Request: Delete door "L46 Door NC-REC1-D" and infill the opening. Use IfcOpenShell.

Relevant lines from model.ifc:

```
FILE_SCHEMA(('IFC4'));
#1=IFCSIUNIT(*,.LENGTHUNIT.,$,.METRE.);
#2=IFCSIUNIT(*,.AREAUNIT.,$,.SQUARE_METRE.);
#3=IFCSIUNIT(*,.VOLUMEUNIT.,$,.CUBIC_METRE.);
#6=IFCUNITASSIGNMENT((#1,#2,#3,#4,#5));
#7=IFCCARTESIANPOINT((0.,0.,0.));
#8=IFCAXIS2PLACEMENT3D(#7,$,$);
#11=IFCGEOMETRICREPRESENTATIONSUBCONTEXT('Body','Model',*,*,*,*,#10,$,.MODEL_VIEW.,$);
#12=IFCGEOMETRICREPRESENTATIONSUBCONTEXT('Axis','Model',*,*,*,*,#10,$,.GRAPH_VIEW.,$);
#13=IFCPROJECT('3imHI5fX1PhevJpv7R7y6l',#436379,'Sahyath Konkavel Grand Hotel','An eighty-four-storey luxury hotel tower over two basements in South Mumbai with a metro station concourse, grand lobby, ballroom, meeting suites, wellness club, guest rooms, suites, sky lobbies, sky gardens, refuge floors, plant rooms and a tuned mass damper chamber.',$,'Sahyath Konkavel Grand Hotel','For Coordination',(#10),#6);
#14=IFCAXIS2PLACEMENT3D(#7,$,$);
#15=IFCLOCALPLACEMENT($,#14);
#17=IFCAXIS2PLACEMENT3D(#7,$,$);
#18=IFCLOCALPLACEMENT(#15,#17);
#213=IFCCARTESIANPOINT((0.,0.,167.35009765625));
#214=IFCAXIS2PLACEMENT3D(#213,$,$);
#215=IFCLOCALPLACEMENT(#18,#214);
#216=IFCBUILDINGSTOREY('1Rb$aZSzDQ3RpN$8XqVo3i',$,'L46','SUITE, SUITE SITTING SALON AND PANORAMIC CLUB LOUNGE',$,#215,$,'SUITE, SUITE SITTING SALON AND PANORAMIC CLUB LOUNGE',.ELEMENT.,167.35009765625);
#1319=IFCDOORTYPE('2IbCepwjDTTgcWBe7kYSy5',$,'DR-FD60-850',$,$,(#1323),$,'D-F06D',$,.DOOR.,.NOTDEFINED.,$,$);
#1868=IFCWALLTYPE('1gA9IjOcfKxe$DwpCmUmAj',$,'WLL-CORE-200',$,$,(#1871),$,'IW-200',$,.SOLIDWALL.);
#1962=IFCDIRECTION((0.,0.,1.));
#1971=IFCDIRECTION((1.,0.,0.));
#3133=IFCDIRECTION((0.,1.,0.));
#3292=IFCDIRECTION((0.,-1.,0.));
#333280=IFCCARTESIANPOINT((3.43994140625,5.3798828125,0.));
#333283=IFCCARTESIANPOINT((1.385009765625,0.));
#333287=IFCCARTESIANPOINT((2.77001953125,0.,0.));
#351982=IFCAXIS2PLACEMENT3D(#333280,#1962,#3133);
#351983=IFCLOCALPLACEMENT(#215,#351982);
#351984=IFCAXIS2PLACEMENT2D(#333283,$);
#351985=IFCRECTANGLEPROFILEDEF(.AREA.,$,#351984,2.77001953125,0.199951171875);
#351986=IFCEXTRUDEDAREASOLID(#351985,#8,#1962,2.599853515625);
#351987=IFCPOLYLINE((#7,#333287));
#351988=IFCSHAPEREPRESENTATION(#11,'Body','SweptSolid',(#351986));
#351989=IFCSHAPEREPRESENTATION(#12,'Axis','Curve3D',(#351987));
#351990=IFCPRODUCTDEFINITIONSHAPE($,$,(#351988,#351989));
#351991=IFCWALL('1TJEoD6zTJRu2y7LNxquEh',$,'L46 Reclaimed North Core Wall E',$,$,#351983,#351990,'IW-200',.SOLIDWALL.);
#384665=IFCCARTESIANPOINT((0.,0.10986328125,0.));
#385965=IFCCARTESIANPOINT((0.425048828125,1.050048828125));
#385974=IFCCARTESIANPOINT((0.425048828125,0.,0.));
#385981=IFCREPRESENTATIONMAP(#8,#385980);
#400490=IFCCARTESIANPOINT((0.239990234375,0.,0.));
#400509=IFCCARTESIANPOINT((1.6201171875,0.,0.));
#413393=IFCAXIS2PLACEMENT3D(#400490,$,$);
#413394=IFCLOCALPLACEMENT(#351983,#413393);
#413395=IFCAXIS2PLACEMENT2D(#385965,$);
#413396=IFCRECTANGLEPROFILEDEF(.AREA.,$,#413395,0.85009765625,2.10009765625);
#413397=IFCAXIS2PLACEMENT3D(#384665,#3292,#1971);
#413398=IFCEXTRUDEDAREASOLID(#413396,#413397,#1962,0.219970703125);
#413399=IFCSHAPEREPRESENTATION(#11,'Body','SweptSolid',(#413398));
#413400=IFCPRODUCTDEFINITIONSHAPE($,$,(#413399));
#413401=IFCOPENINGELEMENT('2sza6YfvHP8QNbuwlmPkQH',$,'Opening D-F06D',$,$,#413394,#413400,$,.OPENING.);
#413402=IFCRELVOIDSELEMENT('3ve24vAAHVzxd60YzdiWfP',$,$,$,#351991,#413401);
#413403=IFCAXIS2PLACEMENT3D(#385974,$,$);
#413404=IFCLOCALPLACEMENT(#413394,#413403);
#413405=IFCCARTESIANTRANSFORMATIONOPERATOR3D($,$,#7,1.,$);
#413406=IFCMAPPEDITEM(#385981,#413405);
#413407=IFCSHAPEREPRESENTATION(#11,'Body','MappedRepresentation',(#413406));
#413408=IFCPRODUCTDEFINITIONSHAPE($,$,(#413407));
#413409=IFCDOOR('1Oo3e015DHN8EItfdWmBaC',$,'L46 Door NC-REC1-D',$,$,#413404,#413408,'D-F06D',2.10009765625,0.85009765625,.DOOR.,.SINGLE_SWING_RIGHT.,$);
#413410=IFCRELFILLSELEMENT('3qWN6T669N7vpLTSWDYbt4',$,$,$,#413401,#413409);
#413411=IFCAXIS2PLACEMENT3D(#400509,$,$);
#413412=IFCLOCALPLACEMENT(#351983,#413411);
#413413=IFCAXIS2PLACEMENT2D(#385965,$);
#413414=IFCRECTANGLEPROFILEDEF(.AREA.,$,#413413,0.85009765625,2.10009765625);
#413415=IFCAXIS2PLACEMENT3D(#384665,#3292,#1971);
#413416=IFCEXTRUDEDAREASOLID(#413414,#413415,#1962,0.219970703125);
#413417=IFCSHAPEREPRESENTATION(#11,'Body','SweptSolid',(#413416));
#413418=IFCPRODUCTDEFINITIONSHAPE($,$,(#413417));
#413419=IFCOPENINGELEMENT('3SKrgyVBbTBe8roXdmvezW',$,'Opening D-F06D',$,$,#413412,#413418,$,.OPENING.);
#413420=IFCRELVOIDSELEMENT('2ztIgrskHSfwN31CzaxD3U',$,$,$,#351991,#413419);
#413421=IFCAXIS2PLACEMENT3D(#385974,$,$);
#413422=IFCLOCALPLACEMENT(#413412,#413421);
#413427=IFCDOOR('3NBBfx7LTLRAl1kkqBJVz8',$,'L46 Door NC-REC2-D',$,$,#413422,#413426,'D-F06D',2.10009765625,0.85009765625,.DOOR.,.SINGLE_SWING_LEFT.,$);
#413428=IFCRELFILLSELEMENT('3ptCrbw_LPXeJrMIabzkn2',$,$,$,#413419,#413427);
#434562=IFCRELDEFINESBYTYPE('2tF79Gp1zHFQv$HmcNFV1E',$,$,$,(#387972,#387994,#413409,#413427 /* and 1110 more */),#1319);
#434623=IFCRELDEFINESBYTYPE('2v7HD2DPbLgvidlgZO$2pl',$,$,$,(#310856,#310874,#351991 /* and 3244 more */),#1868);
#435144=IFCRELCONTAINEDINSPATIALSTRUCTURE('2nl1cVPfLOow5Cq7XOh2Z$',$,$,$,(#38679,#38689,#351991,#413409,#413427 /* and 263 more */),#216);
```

```python
import ifcopenshell
import ifcopenshell.api.feature
import ifcopenshell.api.root
import ifcopenshell.geom
import ifcopenshell.util.shape

model = ifcopenshell.open("model.ifc")
settings = ifcopenshell.geom.settings()


def volume(element):
    """Net volume in cubic metres, openings subtracted."""
    shape = ifcopenshell.geom.create_shape(settings, element)
    return ifcopenshell.util.shape.get_volume(shape.geometry)


door = model.by_id(413409)
opening = door.FillsVoids[0].RelatingOpeningElement
wall = opening.VoidsElements[0].RelatingBuildingElement
before = volume(wall)

ifcopenshell.api.root.remove_product(model, product=door)
ifcopenshell.api.feature.remove_feature(model, feature=opening)

after = volume(wall)

print(f"wall volume {before:.3f} -> {after:.3f} m3")

model.write("model_updated.ifc")
```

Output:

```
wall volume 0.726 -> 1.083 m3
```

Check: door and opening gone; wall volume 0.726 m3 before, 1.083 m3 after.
